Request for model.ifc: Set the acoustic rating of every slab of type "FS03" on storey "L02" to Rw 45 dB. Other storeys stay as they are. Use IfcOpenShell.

First a look at what the model holds.

```python
import ifcopenshell
import ifcopenshell.util.element

model = ifcopenshell.open("model.ifc")
print(model.schema)
storey = next(s for s in model.by_type("IfcBuildingStorey") if s.Name == "L02")
slabs = [e for e in ifcopenshell.util.element.get_decomposition(storey) if e.is_a("IfcSlab")]
seen = {}
for e in slabs:
    element_type = ifcopenshell.util.element.get_type(e)
    key = (element_type.Name if element_type != e and element_type else None, ifcopenshell.util.element.get_pset(e, "Pset_SlabCommon", "AcousticRating"))
    seen[key] = seen.get(key, 0) + 1
for (name, value), count in sorted(seen.items(), key=str):
    print(count, "x", name, "|", value)
```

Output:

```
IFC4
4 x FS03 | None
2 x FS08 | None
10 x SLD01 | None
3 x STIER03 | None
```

```python
import ifcopenshell
import ifcopenshell.api.pset
import ifcopenshell.util.element

model = ifcopenshell.open("model.ifc")

storey = next(s for s in model.by_type("IfcBuildingStorey") if s.Name == "L02")
slabs = [e for e in ifcopenshell.util.element.get_decomposition(storey) if e.is_a("IfcSlab")]

count = 0
for e in slabs:
    element_type = ifcopenshell.util.element.get_type(e)
    if element_type in (None, e) or element_type.Name != "FS03":
        continue
    # add_pset returns the element's existing set when there is one.
    pset = ifcopenshell.api.pset.add_pset(model, product=e, name="Pset_SlabCommon")
    ifcopenshell.api.pset.edit_pset(model, pset=pset, properties={"AcousticRating": "Rw 45 dB"})
    count += 1

print(count, "slabs updated")

model.write("model-out.ifc")
```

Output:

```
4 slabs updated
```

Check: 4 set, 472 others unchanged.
